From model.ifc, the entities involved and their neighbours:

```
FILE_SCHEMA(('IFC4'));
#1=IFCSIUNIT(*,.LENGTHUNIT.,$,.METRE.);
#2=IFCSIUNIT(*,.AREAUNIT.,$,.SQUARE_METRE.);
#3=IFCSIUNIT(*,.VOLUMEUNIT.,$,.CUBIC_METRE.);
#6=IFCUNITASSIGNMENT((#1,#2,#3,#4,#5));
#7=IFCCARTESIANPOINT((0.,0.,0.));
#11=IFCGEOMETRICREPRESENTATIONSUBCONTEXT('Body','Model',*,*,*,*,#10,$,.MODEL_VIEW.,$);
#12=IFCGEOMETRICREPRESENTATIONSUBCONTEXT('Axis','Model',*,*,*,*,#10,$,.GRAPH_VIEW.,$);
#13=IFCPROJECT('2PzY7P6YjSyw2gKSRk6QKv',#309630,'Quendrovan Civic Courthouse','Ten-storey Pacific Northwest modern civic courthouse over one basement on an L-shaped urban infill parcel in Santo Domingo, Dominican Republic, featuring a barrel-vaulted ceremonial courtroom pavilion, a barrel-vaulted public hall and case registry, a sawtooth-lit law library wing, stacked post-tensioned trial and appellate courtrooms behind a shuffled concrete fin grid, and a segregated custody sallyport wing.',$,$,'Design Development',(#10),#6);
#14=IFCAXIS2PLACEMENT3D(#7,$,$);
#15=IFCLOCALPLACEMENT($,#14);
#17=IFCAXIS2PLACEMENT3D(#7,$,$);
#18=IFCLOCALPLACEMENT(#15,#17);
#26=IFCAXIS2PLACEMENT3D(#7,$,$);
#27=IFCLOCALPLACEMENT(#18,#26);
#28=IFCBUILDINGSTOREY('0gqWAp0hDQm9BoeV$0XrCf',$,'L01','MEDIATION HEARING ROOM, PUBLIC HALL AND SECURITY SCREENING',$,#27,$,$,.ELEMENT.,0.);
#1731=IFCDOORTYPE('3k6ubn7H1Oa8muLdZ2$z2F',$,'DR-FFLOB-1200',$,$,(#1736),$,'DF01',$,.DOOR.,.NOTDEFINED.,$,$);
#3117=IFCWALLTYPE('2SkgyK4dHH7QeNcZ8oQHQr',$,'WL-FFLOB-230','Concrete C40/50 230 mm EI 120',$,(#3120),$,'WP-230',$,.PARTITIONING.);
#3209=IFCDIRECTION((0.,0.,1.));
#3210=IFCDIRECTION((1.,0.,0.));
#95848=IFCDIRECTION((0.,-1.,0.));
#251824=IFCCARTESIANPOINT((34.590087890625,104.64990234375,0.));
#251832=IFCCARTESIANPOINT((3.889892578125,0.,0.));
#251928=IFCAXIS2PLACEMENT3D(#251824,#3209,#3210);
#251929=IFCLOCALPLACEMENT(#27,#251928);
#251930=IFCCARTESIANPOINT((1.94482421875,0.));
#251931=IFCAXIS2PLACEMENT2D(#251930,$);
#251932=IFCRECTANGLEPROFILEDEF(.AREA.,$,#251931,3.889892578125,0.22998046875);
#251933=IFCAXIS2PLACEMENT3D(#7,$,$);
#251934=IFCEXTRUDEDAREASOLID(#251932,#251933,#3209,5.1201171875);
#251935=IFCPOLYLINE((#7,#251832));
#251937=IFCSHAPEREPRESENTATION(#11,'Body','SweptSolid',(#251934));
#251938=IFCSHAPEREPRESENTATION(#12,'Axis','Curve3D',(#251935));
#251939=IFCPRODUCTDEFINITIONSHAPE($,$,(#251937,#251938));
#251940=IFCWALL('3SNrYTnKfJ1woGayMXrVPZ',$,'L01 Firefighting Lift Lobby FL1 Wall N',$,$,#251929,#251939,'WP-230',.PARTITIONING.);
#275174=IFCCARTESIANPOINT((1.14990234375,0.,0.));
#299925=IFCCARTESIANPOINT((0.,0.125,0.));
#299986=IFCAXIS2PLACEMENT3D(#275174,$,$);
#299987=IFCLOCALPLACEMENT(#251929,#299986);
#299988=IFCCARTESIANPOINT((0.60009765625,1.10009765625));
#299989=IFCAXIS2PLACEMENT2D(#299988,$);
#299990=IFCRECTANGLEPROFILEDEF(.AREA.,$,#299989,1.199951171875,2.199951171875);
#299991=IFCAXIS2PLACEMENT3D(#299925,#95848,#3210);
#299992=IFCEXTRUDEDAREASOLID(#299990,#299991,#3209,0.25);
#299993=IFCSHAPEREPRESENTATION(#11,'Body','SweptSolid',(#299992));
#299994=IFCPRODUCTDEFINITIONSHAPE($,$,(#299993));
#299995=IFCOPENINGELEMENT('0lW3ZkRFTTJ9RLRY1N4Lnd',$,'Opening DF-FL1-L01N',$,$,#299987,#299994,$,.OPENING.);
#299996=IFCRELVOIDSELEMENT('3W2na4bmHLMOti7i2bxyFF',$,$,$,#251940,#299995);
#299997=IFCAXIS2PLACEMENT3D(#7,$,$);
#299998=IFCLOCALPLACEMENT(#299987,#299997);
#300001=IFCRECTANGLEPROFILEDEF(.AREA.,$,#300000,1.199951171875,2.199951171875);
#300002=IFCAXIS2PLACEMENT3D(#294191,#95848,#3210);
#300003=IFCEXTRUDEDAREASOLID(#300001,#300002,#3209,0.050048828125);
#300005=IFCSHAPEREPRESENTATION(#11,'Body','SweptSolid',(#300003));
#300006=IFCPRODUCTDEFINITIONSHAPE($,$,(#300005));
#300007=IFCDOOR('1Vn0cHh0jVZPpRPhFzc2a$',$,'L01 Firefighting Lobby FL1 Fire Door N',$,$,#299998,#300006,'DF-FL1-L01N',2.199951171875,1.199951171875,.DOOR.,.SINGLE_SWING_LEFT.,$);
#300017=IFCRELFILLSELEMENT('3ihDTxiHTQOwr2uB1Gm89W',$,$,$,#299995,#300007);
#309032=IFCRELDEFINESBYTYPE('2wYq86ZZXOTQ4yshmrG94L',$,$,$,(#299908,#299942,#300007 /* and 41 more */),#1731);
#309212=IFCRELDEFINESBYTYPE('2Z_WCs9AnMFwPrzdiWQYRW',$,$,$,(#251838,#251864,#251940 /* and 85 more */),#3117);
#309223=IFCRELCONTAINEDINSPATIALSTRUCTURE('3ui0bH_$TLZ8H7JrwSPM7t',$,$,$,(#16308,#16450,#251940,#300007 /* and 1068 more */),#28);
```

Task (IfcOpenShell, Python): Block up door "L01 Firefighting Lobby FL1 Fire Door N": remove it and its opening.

```python
import ifcopenshell
import ifcopenshell.api.feature
import ifcopenshell.api.root
import ifcopenshell.geom
import ifcopenshell.util.shape

model = ifcopenshell.open("model.ifc")
settings = ifcopenshell.geom.settings()


def volume(element):
    """Net volume in cubic metres, openings subtracted."""
    shape = ifcopenshell.geom.create_shape(settings, element)
    return ifcopenshell.util.shape.get_volume(shape.geometry)


door = model.by_guid("1Vn0cHh0jVZPpRPhFzc2a$")
opening = door.FillsVoids[0].RelatingOpeningElement
wall = opening.VoidsElements[0].RelatingBuildingElement
before = volume(wall)

ifcopenshell.api.root.remove_product(model, product=door)
ifcopenshell.api.feature.remove_feature(model, feature=opening)

after = volume(wall)

print(f"wall volume {before:.3f} -> {after:.3f} m3")

model.write("model_edited.ifc")
```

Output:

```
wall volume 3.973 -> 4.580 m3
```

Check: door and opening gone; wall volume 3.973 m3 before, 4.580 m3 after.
